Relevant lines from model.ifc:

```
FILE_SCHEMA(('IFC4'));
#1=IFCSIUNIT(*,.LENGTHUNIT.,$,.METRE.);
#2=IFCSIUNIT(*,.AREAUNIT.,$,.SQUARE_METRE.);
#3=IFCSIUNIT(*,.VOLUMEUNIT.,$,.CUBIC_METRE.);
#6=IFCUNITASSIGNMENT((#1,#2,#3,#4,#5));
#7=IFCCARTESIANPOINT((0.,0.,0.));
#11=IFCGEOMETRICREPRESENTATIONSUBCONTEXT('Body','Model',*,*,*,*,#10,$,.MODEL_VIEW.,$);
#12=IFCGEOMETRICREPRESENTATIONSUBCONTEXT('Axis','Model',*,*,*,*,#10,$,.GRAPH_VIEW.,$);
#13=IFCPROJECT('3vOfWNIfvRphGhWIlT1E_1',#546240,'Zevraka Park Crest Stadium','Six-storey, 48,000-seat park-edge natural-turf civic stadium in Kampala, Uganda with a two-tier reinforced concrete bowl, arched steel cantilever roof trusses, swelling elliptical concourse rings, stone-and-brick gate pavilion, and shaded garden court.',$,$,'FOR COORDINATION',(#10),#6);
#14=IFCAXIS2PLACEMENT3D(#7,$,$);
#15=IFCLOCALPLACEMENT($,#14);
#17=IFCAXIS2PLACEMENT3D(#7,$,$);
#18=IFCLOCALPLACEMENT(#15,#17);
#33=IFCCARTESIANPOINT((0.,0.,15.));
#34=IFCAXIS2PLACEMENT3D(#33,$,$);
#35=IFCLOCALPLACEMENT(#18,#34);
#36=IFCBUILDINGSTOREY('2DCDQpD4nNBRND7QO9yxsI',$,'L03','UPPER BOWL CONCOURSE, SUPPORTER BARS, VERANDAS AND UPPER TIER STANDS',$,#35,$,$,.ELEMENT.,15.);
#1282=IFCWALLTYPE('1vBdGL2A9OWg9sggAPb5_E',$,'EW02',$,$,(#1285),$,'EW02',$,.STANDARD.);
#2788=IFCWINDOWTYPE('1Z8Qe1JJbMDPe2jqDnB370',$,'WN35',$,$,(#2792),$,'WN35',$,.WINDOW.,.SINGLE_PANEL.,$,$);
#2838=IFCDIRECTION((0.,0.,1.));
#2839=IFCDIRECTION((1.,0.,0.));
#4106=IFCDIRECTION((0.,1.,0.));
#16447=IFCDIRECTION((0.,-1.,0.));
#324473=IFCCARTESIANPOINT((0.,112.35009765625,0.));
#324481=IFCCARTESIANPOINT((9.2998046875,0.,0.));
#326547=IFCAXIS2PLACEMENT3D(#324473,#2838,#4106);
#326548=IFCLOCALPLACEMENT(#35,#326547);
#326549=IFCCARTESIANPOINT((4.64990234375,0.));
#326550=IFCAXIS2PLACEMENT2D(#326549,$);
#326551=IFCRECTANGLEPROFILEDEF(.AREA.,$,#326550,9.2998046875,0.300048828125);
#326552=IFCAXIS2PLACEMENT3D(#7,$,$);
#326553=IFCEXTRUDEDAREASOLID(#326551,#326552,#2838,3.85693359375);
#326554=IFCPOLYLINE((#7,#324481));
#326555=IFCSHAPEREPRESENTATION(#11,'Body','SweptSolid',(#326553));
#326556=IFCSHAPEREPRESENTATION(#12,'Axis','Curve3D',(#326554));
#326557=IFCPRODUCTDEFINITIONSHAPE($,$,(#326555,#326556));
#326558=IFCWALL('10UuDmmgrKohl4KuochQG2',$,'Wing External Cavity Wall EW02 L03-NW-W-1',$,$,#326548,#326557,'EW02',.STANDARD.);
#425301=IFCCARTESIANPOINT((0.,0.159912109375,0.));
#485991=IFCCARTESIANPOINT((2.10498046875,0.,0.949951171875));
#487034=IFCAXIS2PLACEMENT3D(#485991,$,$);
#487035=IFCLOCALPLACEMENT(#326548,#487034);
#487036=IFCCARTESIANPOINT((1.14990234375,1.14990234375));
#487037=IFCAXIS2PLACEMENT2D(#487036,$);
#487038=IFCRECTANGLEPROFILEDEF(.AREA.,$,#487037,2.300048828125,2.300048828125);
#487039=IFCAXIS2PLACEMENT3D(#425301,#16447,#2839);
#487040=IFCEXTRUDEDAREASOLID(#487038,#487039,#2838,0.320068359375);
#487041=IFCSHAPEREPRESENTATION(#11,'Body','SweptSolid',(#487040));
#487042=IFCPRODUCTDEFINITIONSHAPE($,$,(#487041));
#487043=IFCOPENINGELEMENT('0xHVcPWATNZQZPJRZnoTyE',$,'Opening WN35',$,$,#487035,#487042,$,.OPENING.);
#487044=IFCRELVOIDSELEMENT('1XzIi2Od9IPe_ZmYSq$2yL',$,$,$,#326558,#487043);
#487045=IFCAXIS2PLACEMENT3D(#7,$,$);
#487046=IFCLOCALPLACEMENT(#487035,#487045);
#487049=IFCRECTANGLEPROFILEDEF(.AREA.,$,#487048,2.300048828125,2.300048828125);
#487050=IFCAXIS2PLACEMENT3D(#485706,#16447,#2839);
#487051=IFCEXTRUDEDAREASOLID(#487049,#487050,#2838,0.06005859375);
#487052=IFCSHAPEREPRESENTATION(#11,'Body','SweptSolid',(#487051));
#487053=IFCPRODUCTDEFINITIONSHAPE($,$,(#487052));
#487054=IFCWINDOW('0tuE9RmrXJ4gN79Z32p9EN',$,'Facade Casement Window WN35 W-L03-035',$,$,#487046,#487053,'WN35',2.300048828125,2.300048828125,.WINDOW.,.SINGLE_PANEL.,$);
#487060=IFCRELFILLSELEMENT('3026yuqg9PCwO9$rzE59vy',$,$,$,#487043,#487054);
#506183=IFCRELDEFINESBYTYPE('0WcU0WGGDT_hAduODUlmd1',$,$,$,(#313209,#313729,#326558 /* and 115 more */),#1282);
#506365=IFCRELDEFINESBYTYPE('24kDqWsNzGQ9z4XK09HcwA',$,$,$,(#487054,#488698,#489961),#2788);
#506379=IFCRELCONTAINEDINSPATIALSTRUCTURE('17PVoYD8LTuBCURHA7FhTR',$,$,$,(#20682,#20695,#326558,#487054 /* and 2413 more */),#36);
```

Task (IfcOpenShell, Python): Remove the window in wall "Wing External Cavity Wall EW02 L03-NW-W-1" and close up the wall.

```python
import ifcopenshell
import ifcopenshell.api.feature
import ifcopenshell.api.root
import ifcopenshell.geom
import ifcopenshell.util.shape

model = ifcopenshell.open("model.ifc")
settings = ifcopenshell.geom.settings()


def volume(element):
    """Net volume in cubic metres, openings subtracted."""
    shape = ifcopenshell.geom.create_shape(settings, element)
    return ifcopenshell.util.shape.get_volume(shape.geometry)


window = model.by_guid("0tuE9RmrXJ4gN79Z32p9EN")
opening = window.FillsVoids[0].RelatingOpeningElement
wall = opening.VoidsElements[0].RelatingBuildingElement
before = volume(wall)

ifcopenshell.api.root.remove_product(model, product=window)
ifcopenshell.api.feature.remove_feature(model, feature=opening)

after = volume(wall)

print(f"wall volume {before:.3f} -> {after:.3f} m3")

model.write("model_v2.ifc")
```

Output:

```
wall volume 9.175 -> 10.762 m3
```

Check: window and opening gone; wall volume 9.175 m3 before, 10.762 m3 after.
